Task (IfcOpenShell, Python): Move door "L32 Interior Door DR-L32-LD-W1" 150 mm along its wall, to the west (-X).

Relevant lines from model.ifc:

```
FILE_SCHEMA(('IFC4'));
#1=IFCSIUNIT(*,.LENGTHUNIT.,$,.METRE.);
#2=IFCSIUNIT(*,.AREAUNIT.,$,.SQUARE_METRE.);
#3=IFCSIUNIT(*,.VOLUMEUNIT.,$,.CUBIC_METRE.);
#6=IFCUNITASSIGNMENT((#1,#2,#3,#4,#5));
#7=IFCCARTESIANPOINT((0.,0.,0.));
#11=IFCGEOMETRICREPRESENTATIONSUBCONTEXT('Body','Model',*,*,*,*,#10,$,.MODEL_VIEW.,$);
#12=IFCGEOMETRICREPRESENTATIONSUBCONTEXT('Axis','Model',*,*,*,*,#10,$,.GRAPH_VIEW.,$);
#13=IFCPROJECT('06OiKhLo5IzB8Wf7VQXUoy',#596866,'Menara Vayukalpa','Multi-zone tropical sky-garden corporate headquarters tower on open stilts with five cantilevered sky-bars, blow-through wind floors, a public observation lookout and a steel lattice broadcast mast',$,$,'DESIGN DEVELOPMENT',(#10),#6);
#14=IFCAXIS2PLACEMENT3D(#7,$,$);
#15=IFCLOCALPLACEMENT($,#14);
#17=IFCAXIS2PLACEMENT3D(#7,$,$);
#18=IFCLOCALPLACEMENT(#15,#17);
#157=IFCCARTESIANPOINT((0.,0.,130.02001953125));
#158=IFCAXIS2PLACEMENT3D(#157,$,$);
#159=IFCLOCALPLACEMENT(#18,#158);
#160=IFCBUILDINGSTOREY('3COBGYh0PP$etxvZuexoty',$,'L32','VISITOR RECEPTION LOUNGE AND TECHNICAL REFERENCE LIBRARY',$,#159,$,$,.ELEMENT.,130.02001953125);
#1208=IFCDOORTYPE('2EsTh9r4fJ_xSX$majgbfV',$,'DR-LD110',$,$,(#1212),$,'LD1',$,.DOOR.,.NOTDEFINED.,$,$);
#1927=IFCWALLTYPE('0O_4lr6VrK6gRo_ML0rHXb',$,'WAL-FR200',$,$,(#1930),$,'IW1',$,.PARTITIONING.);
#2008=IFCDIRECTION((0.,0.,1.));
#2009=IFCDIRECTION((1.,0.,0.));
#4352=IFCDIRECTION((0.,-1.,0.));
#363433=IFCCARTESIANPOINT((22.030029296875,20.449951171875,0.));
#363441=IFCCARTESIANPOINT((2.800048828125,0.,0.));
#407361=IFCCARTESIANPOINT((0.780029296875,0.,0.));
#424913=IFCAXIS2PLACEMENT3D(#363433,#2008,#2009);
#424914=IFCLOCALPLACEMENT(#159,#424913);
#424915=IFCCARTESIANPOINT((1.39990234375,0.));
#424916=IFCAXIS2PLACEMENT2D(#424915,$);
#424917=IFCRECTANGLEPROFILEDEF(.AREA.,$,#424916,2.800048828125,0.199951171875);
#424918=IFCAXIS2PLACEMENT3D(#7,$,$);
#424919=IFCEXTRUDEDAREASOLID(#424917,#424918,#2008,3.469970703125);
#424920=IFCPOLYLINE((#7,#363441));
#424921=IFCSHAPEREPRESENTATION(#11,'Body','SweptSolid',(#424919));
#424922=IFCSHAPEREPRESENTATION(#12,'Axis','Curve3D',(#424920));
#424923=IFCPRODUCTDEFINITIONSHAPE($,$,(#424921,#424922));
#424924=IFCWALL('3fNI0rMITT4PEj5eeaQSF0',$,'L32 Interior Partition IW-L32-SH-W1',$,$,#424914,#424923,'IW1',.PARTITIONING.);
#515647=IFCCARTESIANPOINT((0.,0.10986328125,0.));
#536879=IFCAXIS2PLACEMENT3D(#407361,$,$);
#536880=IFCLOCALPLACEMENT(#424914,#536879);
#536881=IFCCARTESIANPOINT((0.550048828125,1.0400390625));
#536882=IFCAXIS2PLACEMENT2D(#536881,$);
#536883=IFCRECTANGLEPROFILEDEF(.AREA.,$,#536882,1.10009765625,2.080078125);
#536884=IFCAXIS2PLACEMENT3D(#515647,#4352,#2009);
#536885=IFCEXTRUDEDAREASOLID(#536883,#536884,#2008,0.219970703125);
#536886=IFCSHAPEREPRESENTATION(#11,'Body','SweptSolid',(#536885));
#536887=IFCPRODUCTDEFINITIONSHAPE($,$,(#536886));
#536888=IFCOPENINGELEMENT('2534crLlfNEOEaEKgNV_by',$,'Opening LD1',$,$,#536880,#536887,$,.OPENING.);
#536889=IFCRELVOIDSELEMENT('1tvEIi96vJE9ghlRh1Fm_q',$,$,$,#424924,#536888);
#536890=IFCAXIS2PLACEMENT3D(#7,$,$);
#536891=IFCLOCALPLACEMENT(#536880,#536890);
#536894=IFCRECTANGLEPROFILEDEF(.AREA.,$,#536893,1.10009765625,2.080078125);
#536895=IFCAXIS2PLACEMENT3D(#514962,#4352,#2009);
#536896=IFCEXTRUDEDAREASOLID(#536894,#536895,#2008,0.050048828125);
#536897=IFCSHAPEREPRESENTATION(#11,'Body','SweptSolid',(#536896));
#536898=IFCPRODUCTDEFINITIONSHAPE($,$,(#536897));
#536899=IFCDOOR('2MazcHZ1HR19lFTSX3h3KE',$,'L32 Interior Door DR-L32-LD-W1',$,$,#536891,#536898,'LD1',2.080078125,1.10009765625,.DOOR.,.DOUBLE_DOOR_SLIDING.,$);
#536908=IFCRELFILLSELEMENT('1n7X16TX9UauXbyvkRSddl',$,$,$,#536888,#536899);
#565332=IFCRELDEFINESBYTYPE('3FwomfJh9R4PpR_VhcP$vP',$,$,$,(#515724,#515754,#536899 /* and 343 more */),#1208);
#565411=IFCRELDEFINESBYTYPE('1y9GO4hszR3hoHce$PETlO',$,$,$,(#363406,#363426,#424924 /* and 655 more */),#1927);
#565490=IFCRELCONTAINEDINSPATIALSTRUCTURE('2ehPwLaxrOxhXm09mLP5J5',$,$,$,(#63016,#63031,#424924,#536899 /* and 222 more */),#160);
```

```python
import ifcopenshell
import ifcopenshell.api.geometry
import ifcopenshell.util.placement
import ifcopenshell.util.unit

model = ifcopenshell.open("model.ifc")
unit_scale = ifcopenshell.util.unit.calculate_unit_scale(model)

door = model.by_guid("2MazcHZ1HR19lFTSX3h3KE")
opening = door.FillsVoids[0].RelatingOpeningElement
wall = opening.VoidsElements[0].RelatingBuildingElement

wall_matrix = ifcopenshell.util.placement.get_local_placement(wall.ObjectPlacement)
shift = wall_matrix[:3, 0] * -0.15 / unit_scale
before = ifcopenshell.util.placement.get_local_placement(door.ObjectPlacement)[:3, 3].copy()

# The door is placed relative to its opening, so it follows when the opening moves.
matrix = ifcopenshell.util.placement.get_local_placement(opening.ObjectPlacement)
matrix[:3, 3] += shift
ifcopenshell.api.geometry.edit_object_placement(
    model, product=opening, matrix=matrix, is_si=False, should_transform_children=True
)

after = ifcopenshell.util.placement.get_local_placement(door.ObjectPlacement)[:3, 3]
print("door moved by", (after - before).round(3) + 0.0)

model.write("model-out.ifc")
```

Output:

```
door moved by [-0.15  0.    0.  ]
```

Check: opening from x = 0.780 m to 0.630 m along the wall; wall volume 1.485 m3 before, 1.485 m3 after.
